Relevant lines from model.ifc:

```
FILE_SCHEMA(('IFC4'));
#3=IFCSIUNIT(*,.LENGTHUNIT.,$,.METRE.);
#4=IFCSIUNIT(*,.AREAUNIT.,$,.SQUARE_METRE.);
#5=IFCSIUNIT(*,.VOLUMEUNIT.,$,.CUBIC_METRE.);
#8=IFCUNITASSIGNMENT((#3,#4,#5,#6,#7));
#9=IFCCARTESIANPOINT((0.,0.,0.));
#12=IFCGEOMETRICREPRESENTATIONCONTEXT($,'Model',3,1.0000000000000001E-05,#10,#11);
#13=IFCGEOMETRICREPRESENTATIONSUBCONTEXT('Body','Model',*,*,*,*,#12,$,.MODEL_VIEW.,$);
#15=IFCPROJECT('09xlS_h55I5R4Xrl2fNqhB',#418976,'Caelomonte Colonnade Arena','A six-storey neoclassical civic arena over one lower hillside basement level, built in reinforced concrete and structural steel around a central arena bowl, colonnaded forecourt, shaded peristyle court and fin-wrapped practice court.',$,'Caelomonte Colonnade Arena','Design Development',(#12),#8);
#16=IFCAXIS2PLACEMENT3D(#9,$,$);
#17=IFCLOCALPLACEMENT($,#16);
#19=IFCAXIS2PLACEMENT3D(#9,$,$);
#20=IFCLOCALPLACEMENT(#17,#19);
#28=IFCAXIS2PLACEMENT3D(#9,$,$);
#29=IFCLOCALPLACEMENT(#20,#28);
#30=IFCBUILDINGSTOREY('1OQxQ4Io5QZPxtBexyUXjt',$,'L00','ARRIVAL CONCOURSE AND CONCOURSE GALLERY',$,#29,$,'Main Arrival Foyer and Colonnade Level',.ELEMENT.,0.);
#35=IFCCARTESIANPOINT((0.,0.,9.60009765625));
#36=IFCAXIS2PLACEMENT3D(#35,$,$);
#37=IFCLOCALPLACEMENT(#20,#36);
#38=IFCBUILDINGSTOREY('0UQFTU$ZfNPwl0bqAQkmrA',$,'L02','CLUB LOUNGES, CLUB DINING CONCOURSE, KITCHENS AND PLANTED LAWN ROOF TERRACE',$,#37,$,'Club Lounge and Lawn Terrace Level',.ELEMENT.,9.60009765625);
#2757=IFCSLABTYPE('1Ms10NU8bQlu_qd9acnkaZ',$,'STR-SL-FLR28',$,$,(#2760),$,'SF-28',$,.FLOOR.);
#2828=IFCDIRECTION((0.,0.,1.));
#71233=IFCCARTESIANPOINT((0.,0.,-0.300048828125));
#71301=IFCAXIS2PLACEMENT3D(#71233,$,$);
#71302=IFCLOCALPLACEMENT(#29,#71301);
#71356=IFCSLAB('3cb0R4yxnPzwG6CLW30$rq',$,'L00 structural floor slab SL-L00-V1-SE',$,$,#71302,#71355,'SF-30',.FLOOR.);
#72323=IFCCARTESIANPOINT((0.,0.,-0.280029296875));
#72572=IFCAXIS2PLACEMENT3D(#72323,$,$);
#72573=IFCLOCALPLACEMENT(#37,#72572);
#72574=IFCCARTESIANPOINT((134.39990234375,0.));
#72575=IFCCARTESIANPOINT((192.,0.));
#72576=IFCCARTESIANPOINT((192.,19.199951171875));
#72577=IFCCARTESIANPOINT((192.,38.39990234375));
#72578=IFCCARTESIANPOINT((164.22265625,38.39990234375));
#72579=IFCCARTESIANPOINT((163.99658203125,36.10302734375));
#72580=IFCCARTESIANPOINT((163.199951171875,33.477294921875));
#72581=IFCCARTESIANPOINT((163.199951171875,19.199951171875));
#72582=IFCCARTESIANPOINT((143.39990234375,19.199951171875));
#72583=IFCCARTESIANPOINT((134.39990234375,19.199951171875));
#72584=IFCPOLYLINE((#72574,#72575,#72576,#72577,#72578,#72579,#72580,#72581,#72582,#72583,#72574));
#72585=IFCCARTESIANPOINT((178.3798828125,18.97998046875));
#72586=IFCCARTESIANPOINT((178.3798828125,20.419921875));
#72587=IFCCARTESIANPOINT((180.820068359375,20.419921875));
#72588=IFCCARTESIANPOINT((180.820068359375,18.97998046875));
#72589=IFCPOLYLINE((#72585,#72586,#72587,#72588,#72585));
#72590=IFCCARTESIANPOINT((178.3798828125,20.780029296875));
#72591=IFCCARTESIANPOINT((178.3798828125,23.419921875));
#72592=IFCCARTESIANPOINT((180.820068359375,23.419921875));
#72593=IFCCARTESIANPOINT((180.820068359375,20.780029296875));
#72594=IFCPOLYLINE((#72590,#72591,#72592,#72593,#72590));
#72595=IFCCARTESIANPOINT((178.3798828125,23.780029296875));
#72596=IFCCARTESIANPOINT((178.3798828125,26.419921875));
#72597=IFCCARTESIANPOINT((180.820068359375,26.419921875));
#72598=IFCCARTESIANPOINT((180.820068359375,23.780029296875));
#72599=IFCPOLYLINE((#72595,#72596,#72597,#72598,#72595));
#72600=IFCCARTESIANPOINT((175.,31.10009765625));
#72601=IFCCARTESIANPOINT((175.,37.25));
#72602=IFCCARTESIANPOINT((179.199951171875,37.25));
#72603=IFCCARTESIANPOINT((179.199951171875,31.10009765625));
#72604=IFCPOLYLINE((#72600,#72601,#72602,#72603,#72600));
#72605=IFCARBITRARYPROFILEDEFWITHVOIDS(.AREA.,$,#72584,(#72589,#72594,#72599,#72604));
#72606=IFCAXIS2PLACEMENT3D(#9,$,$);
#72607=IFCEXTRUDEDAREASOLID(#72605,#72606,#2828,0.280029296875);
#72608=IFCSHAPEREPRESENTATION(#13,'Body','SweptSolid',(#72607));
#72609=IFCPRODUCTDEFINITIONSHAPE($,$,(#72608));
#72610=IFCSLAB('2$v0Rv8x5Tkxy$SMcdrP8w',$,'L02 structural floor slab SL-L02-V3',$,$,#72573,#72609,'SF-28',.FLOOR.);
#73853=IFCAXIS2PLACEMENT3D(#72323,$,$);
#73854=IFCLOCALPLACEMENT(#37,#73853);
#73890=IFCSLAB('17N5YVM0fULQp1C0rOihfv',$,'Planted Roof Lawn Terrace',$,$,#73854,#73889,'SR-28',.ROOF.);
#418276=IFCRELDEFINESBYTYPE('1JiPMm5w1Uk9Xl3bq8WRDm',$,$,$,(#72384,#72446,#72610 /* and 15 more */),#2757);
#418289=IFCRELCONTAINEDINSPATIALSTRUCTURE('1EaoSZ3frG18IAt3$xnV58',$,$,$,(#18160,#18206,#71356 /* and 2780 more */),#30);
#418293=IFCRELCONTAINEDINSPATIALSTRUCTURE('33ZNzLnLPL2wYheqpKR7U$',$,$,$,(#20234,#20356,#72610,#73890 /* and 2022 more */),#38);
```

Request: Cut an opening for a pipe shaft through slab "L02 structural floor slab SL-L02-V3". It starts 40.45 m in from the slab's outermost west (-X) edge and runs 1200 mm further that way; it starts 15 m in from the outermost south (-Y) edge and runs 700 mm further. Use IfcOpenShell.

```python
import numpy as np
import ifcopenshell
import ifcopenshell.api.feature
import ifcopenshell.api.geometry
import ifcopenshell.api.root
import ifcopenshell.geom
import ifcopenshell.util.placement
import ifcopenshell.util.representation
import ifcopenshell.util.shape
import ifcopenshell.util.unit

model = ifcopenshell.open("model.ifc")
unit_scale = ifcopenshell.util.unit.calculate_unit_scale(model)
settings = ifcopenshell.geom.settings()


def volume(element):
    """Net volume in cubic metres, openings subtracted."""
    shape = ifcopenshell.geom.create_shape(settings, element)
    return ifcopenshell.util.shape.get_volume(shape.geometry)


slab = model.by_guid("2$v0Rv8x5Tkxy$SMcdrP8w")
before = volume(slab)

# Extent in the slab's own axes, in metres. The edges named are its -X and -Y sides.
slab_shape = ifcopenshell.geom.create_shape(settings, slab)
vertices = ifcopenshell.util.shape.get_vertices(slab_shape.geometry)
x_min, y_min, bottom = vertices.min(axis=0)
top = vertices[:, 2].max()

opening = ifcopenshell.api.root.create_entity(model, ifc_class="IfcOpeningElement", name="Pipe shaft opening", predefined_type="OPENING")
context = ifcopenshell.util.representation.get_context(model, "Model", "Body", "MODEL_VIEW")
width, depth = 1.2, 0.7
outline = [(0.0, 0.0), (width, 0.0), (width, depth), (0.0, depth), (0.0, 0.0)]
# Overshoot both faces by 50 mm so the cut is clean.
shape = ifcopenshell.api.geometry.add_slab_representation(
    model, context=context, depth=top - bottom + 0.1, polyline=outline
)
ifcopenshell.api.geometry.assign_representation(model, product=opening, representation=shape)

matrix = ifcopenshell.util.placement.get_local_placement(slab.ObjectPlacement)
matrix[:, 3] = matrix @ np.append(np.array([x_min + 40.45, y_min + 15, bottom - 0.05]) / unit_scale, 1.0)
ifcopenshell.api.geometry.edit_object_placement(model, product=opening, matrix=matrix, is_si=False)
ifcopenshell.api.feature.add_feature(model, feature=opening, element=slab)

after = volume(slab)

print(f"slab volume {before:.3f} -> {after:.3f} m3")

model.write("model-out.ifc")
```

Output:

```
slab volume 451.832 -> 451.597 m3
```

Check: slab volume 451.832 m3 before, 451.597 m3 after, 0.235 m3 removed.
